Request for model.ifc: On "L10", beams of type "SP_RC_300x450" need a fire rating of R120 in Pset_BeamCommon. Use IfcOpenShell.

First a look at what the model holds.

```python
import ifcopenshell
import ifcopenshell.util.element

model = ifcopenshell.open("model.ifc")
print(model.schema)
storey = next(s for s in model.by_type("IfcBuildingStorey") if s.Name == "L10")
beams = [e for e in ifcopenshell.util.element.get_decomposition(storey) if e.is_a("IfcBeam")]
seen = {}
for e in beams:
    element_type = ifcopenshell.util.element.get_type(e)
    key = (element_type.Name if element_type != e and element_type else None, ifcopenshell.util.element.get_pset(e, "Pset_BeamCommon", "FireRating"))
    seen[key] = seen.get(key, 0) + 1
for (name, value), count in sorted(seen.items(), key=str):
    print(count, "x", name, "|", value)
```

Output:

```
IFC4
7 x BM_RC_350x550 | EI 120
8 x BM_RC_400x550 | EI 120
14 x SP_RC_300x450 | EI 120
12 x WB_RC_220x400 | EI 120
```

```python
import ifcopenshell
import ifcopenshell.api.pset
import ifcopenshell.util.element

model = ifcopenshell.open("model.ifc")

storey = next(s for s in model.by_type("IfcBuildingStorey") if s.Name == "L10")
beams = [e for e in ifcopenshell.util.element.get_decomposition(storey) if e.is_a("IfcBeam")]

count = 0
for e in beams:
    element_type = ifcopenshell.util.element.get_type(e)
    if element_type in (None, e) or element_type.Name != "SP_RC_300x450":
        continue
    # add_pset returns the element's existing set when there is one.
    pset = ifcopenshell.api.pset.add_pset(model, product=e, name="Pset_BeamCommon")
    ifcopenshell.api.pset.edit_pset(model, pset=pset, properties={"FireRating": "R120"})
    count += 1

print(count, "beams updated")

model.write("model_edited.ifc")
```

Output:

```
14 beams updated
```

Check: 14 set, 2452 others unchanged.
